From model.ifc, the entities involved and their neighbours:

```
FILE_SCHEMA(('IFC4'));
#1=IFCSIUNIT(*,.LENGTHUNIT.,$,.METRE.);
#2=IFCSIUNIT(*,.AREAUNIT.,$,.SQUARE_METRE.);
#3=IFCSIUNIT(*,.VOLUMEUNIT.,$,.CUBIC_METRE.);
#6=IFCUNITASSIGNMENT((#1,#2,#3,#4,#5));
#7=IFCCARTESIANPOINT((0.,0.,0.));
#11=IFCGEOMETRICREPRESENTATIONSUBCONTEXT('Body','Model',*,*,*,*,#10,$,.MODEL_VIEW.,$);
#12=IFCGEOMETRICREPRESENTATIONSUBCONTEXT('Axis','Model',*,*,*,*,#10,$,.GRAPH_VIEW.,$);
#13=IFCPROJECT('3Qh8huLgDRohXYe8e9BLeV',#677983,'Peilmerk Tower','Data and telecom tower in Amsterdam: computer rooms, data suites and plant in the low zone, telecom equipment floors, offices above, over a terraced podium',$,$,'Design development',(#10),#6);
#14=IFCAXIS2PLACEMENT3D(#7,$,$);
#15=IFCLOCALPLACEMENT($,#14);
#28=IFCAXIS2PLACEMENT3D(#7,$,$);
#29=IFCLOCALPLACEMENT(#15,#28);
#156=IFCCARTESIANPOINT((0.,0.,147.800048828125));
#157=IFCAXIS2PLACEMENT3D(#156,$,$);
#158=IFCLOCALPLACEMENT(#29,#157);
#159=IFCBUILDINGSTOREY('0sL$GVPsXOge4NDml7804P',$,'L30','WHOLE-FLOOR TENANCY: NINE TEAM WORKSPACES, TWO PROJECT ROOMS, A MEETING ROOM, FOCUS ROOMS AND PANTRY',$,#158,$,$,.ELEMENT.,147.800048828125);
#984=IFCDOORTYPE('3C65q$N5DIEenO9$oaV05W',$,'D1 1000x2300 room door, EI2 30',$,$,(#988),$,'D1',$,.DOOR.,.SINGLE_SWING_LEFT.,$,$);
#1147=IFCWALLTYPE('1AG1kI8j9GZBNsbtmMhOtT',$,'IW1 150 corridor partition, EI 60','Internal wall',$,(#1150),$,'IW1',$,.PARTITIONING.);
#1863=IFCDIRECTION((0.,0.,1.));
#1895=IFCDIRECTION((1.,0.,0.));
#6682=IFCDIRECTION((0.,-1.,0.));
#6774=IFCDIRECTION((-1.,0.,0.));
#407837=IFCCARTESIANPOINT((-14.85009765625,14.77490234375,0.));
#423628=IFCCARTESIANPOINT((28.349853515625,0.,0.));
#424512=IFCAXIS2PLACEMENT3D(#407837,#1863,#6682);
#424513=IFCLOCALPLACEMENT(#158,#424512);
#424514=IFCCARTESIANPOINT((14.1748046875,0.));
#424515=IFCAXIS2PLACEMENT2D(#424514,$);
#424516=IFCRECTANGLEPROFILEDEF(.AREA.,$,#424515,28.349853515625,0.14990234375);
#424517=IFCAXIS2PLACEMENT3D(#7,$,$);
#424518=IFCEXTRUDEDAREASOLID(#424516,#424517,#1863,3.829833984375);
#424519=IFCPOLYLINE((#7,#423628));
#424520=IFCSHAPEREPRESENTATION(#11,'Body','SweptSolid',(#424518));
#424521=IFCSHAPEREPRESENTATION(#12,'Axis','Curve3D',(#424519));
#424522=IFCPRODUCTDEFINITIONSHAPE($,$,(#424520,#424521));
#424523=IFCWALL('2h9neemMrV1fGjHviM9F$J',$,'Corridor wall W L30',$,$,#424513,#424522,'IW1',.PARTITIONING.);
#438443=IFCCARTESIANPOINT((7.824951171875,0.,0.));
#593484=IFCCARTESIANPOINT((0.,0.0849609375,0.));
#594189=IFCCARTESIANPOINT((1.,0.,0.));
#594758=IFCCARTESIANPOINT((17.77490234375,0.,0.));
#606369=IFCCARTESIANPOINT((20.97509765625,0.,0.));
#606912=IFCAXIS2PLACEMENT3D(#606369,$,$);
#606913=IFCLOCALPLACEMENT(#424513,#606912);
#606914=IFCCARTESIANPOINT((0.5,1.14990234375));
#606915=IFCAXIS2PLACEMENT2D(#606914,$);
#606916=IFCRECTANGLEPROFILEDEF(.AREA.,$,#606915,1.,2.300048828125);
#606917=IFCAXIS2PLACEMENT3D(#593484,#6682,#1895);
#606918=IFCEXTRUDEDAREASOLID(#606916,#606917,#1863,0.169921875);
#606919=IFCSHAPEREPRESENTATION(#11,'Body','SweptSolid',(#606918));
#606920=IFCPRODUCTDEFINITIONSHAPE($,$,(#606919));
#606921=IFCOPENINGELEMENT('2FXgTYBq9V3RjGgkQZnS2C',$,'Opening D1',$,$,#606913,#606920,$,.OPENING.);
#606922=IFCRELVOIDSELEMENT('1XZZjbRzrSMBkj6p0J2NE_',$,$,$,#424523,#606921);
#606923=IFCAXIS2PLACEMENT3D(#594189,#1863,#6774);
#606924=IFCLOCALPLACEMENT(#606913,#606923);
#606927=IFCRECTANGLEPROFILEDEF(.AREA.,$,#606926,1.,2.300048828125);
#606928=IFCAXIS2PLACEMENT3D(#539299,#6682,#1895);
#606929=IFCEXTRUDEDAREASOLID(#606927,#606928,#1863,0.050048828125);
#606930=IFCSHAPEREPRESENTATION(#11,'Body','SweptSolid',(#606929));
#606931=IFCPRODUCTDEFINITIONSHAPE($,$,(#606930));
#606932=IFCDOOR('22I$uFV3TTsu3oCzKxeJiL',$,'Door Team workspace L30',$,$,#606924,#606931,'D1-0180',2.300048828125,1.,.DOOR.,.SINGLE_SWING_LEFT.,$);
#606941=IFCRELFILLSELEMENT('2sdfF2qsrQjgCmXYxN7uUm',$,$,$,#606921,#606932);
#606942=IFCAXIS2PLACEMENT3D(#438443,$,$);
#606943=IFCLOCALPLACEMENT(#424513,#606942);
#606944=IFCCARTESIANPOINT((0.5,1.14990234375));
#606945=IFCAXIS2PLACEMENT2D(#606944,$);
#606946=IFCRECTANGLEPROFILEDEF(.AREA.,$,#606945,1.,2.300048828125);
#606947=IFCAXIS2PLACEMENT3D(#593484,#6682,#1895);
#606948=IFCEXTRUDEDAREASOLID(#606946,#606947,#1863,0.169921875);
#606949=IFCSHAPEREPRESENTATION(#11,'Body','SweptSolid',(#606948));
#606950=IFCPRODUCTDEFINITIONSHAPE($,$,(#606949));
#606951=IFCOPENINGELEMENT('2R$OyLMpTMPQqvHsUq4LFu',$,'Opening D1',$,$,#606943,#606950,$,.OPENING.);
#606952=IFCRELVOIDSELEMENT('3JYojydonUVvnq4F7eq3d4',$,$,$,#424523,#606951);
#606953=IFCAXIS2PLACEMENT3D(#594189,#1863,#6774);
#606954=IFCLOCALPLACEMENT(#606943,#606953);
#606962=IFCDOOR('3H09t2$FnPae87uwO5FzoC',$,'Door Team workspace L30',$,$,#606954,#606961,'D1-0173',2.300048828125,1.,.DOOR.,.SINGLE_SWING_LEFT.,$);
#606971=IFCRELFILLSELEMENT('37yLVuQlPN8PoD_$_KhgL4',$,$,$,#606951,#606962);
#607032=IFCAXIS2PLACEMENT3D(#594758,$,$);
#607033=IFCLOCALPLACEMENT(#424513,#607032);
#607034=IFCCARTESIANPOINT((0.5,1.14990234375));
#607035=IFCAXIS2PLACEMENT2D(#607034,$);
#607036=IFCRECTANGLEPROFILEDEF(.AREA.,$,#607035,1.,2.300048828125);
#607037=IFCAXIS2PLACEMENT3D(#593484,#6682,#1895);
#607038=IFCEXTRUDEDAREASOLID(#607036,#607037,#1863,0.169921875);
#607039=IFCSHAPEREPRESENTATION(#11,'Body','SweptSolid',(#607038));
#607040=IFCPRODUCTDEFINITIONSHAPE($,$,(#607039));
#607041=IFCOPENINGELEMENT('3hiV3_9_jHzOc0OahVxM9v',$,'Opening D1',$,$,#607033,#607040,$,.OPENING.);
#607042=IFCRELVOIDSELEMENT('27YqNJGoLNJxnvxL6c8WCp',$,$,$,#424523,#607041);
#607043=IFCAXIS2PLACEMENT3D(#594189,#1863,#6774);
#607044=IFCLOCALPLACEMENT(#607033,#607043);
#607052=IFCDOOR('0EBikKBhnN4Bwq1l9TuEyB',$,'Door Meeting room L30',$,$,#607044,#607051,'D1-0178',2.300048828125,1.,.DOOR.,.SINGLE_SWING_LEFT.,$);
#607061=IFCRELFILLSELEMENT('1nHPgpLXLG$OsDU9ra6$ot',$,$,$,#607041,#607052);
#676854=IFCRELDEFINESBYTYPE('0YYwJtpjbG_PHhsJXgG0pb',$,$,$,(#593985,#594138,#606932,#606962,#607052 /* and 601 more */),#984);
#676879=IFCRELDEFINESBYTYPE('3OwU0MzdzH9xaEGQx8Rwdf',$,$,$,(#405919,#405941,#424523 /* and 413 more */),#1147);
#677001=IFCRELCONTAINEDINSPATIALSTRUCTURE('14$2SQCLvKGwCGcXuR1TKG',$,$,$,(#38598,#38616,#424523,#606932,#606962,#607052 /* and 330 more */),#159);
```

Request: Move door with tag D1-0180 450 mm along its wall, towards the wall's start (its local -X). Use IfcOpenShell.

```python
import ifcopenshell
import ifcopenshell.api.geometry
import ifcopenshell.util.placement
import ifcopenshell.util.unit

model = ifcopenshell.open("model.ifc")
unit_scale = ifcopenshell.util.unit.calculate_unit_scale(model)

door = model.by_guid("22I$uFV3TTsu3oCzKxeJiL")
opening = door.FillsVoids[0].RelatingOpeningElement
wall = opening.VoidsElements[0].RelatingBuildingElement

wall_matrix = ifcopenshell.util.placement.get_local_placement(wall.ObjectPlacement)
shift = wall_matrix[:3, 0] * -0.45 / unit_scale
before = ifcopenshell.util.placement.get_local_placement(door.ObjectPlacement)[:3, 3].copy()

# The door is placed relative to its opening, so it follows when the opening moves.
matrix = ifcopenshell.util.placement.get_local_placement(opening.ObjectPlacement)
matrix[:3, 3] += shift
ifcopenshell.api.geometry.edit_object_placement(
    model, product=opening, matrix=matrix, is_si=False, should_transform_children=True
)

after = ifcopenshell.util.placement.get_local_placement(door.ObjectPlacement)[:3, 3]
print("door moved by", (after - before).round(3) + 0.0)

model.write("model-out.ifc")
```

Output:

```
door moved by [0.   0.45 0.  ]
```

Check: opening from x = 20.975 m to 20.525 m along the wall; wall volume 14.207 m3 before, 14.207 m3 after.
